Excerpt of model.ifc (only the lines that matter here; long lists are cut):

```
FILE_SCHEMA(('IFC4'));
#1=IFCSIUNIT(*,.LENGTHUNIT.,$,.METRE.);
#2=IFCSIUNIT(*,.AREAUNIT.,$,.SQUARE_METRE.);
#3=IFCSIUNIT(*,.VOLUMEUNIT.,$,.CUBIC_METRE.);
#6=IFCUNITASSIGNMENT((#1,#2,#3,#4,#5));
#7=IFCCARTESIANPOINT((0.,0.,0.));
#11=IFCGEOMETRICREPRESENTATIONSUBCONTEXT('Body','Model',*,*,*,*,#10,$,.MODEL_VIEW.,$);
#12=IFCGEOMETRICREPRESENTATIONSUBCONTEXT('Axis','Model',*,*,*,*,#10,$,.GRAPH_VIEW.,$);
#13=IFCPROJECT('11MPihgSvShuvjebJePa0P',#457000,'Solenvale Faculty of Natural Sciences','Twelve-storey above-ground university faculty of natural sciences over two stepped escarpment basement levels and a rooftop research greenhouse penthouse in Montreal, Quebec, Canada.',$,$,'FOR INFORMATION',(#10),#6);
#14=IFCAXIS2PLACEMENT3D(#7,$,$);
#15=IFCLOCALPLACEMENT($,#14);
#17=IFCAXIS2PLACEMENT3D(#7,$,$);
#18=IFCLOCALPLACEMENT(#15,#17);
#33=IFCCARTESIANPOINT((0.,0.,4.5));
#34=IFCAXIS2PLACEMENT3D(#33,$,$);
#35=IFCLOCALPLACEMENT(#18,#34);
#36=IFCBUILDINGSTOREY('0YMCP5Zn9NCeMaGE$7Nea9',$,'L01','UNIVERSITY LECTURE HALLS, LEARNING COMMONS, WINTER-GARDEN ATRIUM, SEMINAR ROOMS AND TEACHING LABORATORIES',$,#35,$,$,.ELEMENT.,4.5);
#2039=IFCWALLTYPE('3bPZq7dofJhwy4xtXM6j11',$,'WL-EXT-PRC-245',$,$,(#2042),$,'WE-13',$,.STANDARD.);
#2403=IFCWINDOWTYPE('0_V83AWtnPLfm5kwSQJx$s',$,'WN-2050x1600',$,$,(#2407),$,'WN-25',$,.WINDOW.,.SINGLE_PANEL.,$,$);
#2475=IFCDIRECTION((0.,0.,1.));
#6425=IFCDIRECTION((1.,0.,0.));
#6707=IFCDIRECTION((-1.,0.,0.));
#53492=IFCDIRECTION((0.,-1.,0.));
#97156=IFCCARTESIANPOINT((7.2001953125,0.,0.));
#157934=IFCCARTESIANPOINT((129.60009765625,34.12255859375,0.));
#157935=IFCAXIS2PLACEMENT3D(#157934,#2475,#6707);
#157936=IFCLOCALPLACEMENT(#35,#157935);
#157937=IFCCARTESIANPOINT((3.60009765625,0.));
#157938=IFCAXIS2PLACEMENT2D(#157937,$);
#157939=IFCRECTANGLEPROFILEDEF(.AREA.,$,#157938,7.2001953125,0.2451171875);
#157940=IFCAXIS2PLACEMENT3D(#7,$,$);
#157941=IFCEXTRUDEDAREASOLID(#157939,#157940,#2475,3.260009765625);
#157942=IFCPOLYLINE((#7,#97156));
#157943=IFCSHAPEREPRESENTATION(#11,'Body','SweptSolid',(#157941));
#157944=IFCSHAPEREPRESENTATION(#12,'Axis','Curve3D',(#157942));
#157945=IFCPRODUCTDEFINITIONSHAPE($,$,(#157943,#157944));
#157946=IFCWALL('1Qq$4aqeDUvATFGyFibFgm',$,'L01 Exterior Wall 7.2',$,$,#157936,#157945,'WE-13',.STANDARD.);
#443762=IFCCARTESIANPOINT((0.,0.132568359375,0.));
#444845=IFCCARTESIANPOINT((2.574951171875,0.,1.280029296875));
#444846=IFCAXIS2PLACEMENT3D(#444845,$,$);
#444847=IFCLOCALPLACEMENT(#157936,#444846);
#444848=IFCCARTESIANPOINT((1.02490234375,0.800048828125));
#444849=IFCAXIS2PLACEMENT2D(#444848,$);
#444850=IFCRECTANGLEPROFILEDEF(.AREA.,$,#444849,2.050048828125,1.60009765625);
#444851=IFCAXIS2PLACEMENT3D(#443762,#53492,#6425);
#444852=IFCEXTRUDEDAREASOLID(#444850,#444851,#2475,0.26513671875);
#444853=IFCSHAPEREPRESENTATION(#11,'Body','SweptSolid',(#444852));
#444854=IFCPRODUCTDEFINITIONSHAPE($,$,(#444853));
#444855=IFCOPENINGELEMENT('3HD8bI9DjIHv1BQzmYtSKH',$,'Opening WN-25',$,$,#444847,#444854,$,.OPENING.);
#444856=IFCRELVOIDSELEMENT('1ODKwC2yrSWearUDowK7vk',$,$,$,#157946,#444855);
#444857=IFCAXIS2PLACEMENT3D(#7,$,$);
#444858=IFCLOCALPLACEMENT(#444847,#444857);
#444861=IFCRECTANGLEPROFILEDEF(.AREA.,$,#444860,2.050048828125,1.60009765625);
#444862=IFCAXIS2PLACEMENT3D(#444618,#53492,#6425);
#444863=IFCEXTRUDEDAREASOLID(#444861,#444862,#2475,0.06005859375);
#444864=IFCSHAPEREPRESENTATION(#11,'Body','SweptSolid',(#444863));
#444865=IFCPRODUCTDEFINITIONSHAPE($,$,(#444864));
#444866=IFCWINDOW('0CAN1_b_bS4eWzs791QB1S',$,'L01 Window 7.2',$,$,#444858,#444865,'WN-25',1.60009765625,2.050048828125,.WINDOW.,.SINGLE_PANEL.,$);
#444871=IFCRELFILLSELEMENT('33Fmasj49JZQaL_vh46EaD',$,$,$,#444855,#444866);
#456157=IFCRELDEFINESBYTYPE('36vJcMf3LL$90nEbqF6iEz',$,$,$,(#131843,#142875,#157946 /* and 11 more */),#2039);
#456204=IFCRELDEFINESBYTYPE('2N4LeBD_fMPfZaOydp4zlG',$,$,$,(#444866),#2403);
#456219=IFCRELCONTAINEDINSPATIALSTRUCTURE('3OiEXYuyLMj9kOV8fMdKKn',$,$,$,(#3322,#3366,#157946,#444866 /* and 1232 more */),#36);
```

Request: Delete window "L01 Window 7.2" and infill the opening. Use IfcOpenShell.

```python
import ifcopenshell
import ifcopenshell.api.feature
import ifcopenshell.api.root
import ifcopenshell.geom
import ifcopenshell.util.shape

model = ifcopenshell.open("model.ifc")
settings = ifcopenshell.geom.settings()


def volume(element):
    """Net volume in cubic metres, openings subtracted."""
    shape = ifcopenshell.geom.create_shape(settings, element)
    return ifcopenshell.util.shape.get_volume(shape.geometry)


window = model.by_guid("0CAN1_b_bS4eWzs791QB1S")
opening = window.FillsVoids[0].RelatingOpeningElement
wall = opening.VoidsElements[0].RelatingBuildingElement
before = volume(wall)

ifcopenshell.api.root.remove_product(model, product=window)
ifcopenshell.api.feature.remove_feature(model, feature=opening)

after = volume(wall)

print(f"wall volume {before:.3f} -> {after:.3f} m3")

model.write("model_updated.ifc")
```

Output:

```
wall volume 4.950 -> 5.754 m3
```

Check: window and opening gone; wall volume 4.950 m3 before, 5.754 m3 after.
